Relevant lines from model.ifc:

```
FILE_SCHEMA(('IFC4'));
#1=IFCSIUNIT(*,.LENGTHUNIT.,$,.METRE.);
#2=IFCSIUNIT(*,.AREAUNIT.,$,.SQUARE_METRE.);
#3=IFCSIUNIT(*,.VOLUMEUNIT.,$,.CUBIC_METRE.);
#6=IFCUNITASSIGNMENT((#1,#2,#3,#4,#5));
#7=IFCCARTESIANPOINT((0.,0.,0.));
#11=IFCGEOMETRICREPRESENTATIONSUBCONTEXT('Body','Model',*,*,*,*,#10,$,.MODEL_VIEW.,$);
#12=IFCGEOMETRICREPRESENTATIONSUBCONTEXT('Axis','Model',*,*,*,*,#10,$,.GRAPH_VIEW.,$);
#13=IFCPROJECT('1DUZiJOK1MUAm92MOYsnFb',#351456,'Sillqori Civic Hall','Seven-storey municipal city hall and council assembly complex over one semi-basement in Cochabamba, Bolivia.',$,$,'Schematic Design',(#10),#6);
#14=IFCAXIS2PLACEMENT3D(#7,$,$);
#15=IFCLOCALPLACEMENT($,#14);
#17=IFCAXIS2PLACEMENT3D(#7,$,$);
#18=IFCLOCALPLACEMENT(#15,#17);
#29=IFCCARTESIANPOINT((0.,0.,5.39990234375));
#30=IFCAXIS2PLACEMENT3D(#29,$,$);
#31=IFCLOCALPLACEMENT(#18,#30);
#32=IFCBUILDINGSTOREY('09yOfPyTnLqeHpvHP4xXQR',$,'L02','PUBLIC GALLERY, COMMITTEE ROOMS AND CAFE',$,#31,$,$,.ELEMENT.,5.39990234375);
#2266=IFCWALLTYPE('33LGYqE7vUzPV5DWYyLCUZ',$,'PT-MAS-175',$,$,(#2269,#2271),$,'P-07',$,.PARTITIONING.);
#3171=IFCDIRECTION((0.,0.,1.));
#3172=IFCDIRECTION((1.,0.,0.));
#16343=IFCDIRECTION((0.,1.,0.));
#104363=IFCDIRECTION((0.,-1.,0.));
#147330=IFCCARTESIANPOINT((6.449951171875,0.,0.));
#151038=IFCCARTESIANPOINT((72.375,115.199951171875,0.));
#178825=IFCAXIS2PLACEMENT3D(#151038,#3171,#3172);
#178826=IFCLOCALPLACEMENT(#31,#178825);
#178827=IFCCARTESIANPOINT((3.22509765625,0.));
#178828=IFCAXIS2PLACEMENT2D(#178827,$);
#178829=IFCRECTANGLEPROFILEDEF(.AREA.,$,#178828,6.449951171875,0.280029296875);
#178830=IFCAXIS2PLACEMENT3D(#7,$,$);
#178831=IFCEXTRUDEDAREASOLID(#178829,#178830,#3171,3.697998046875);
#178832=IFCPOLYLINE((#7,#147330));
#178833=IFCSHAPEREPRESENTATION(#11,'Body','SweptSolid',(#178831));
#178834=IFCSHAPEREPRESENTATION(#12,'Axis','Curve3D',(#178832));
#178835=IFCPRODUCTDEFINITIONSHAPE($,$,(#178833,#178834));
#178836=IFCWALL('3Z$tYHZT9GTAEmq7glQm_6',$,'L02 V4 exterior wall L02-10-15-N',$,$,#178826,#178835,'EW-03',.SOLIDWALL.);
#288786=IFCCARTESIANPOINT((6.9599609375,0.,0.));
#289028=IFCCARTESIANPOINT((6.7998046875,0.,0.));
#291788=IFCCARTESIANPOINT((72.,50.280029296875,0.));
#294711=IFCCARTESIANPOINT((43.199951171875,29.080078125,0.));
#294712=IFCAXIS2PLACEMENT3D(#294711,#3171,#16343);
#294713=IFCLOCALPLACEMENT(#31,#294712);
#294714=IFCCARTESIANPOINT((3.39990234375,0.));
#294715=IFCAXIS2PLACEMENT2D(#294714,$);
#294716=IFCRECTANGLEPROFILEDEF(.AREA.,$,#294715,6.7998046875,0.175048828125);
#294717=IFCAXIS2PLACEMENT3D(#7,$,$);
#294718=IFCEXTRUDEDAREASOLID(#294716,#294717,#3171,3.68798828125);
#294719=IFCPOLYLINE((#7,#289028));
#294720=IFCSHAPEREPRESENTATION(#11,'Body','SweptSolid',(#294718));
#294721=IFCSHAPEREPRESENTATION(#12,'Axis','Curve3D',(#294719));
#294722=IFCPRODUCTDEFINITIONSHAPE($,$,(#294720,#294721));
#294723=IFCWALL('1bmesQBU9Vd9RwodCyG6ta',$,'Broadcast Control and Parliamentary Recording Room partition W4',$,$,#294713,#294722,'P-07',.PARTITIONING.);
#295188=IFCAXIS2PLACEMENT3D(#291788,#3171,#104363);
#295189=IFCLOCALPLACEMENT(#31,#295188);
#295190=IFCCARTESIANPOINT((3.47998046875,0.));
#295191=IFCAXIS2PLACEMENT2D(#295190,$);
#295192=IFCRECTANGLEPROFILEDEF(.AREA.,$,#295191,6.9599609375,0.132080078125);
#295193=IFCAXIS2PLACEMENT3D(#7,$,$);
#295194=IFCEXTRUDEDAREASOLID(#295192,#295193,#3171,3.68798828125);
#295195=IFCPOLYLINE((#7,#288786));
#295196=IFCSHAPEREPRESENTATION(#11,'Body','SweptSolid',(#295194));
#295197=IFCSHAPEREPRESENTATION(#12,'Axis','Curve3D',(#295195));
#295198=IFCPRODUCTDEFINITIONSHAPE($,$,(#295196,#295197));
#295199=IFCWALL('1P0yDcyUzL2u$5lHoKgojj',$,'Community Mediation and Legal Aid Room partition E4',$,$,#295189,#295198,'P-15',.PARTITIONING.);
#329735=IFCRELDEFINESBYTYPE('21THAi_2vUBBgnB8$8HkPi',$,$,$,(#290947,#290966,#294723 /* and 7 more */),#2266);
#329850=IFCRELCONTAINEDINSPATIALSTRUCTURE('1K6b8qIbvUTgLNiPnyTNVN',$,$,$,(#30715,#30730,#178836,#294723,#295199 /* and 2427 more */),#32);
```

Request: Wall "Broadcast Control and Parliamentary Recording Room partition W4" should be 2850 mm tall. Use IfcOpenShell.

```python
import ifcopenshell
import ifcopenshell.geom
import ifcopenshell.util.representation
import ifcopenshell.util.shape
import ifcopenshell.util.unit

model = ifcopenshell.open("model.ifc")
unit_scale = ifcopenshell.util.unit.calculate_unit_scale(model)
settings = ifcopenshell.geom.settings()


def volume(element):
    """Net volume in cubic metres, openings subtracted."""
    shape = ifcopenshell.geom.create_shape(settings, element)
    return ifcopenshell.util.shape.get_volume(shape.geometry)


wall = model.by_id(294723)
before = volume(wall)

body = ifcopenshell.util.representation.get_representation(wall, "Model", "Body")
solid = body.Items[0]
old_height = solid.Depth
solid.Depth = 2.85 / unit_scale
after = volume(wall)

print(f"height {old_height:g} -> {solid.Depth:g}, volume {before:.3f} -> {after:.3f} m3")

model.write("model_edited.ifc")
```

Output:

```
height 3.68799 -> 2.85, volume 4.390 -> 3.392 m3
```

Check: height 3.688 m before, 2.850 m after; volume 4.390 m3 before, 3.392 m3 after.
